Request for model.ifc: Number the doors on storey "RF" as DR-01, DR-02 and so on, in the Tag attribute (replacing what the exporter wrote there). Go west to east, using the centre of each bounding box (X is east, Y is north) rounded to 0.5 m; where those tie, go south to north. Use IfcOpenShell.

First a look at what the model holds.

```python
import ifcopenshell
import ifcopenshell.util.element
import ifcopenshell.util.placement

model = ifcopenshell.open("model.ifc")
print(model.schema)
storey = next(s for s in model.by_type("IfcBuildingStorey") if s.Name == "RF")
doors = [e for e in ifcopenshell.util.element.get_decomposition(storey) if e.is_a("IfcDoor")]
for e in sorted(doors, key=lambda e: e.id()):
    origin = ifcopenshell.util.placement.get_local_placement(e.ObjectPlacement)[:3, 3]
    print(e.id(), e.Tag, e.Name, origin.round(2) + 0.0, sep=" | ")
```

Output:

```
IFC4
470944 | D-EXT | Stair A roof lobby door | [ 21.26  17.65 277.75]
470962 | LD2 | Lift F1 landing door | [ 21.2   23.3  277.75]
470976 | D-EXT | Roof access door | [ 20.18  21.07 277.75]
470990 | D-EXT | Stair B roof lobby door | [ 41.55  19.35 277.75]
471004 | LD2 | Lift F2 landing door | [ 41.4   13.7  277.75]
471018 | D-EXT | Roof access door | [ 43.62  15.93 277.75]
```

```python
import ifcopenshell
import ifcopenshell.geom
import ifcopenshell.util.element
import ifcopenshell.util.shape

model = ifcopenshell.open("model.ifc")
settings = ifcopenshell.geom.settings()
settings.set("use-world-coords", True)


def centre(element):
    shape = ifcopenshell.geom.create_shape(settings, element)
    return ifcopenshell.util.shape.get_bbox_centroid(shape.geometry)


storey = next(s for s in model.by_type("IfcBuildingStorey") if s.Name == "RF")
doors = [e for e in ifcopenshell.util.element.get_decomposition(storey) if e.is_a("IfcDoor")]

# Insertion points can sit at a corner or the storey origin, so sort by the geometry (in metres).
centres = {e: centre(e) for e in doors}
doors.sort(key=lambda e: (round(centres[e][0] / 0.5), centres[e][1]))

for i, e in enumerate(doors, start=1):
    number = f"DR-{i:02d}"
    e.Tag = number
    print(e.id(), number)

model.write("model_v2.ifc")
```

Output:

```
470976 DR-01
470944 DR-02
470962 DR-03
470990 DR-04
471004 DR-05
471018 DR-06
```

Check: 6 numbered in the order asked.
